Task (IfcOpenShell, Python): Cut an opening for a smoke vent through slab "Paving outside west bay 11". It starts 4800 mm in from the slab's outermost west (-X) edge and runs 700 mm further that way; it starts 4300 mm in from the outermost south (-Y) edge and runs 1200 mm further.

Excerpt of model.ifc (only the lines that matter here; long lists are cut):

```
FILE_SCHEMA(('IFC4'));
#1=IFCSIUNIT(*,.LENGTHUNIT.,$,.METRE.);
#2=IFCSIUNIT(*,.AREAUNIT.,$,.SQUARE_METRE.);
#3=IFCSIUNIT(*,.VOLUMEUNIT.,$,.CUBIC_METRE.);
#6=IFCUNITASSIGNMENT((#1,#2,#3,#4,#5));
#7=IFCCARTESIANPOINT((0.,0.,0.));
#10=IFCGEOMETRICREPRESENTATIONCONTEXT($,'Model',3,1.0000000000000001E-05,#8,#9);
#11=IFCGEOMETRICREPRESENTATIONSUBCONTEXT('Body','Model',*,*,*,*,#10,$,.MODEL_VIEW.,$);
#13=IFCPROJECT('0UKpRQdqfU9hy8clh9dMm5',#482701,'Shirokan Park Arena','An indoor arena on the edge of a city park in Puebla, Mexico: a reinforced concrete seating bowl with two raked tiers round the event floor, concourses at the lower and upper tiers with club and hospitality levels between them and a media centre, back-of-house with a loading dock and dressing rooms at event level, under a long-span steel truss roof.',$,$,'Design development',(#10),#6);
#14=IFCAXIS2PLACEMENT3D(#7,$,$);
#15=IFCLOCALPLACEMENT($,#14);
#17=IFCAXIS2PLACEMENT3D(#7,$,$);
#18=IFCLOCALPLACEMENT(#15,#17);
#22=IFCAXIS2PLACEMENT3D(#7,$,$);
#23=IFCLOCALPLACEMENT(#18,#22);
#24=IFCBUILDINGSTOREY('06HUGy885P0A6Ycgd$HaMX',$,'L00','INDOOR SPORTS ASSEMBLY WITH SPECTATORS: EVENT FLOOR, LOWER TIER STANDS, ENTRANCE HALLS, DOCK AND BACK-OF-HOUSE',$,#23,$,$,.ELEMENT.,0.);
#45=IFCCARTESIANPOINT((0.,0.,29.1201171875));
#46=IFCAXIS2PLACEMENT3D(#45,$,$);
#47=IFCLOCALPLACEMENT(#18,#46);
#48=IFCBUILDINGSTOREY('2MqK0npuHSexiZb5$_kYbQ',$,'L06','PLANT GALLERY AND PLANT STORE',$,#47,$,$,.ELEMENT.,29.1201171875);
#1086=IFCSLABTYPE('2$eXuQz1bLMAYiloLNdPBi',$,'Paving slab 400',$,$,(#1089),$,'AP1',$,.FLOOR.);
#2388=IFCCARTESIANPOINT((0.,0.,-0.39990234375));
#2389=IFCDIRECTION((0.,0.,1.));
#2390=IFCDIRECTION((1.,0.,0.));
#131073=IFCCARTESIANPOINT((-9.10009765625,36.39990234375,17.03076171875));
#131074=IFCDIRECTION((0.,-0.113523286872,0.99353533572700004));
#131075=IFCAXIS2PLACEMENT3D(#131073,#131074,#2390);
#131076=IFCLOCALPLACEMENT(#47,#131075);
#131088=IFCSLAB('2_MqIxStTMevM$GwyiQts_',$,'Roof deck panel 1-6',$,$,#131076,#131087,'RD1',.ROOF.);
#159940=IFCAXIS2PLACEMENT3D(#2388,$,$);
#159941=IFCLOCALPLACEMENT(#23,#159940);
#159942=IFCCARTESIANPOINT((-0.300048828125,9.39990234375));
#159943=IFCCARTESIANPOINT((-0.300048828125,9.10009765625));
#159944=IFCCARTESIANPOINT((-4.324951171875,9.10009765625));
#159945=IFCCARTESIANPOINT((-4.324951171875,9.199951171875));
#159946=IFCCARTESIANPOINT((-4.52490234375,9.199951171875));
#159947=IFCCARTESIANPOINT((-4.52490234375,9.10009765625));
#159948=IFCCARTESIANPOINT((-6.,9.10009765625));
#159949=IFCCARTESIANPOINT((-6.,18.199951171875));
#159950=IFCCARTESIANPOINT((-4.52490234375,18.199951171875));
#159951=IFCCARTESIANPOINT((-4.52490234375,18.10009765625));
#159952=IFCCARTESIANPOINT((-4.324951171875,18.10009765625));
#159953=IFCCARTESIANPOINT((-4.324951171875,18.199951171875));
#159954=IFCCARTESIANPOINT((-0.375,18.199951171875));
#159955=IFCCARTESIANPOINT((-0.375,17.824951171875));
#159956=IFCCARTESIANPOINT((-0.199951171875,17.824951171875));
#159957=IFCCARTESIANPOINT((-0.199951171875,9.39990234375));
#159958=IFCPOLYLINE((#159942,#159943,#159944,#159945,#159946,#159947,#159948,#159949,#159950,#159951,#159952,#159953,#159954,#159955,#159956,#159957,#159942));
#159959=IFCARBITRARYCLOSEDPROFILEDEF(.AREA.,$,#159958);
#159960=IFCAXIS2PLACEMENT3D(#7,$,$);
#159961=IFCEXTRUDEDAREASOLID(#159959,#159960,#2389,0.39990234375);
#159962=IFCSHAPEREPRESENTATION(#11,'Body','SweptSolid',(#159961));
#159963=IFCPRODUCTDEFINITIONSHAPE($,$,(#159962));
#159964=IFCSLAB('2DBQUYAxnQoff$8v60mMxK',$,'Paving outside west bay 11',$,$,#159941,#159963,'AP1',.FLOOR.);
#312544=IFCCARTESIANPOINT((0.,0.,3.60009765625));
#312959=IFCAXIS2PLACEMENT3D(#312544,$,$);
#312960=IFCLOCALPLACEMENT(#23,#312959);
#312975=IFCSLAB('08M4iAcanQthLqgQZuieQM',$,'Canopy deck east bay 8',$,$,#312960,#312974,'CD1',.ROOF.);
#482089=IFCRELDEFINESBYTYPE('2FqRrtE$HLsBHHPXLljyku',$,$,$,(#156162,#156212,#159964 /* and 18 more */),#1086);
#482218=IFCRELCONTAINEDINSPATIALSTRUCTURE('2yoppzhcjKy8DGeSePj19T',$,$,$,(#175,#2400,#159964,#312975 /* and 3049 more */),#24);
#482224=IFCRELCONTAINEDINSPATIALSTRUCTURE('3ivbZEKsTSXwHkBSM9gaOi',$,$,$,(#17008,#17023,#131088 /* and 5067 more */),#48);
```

```python
import numpy as np
import ifcopenshell
import ifcopenshell.api.feature
import ifcopenshell.api.geometry
import ifcopenshell.api.root
import ifcopenshell.geom
import ifcopenshell.util.placement
import ifcopenshell.util.representation
import ifcopenshell.util.shape
import ifcopenshell.util.unit

model = ifcopenshell.open("model.ifc")
unit_scale = ifcopenshell.util.unit.calculate_unit_scale(model)
settings = ifcopenshell.geom.settings()


def volume(element):
    """Net volume in cubic metres, openings subtracted."""
    shape = ifcopenshell.geom.create_shape(settings, element)
    return ifcopenshell.util.shape.get_volume(shape.geometry)


slab = model.by_id(159964)
before = volume(slab)

# Extent in the slab's own axes, in metres. The edges named are its -X and -Y sides.
slab_shape = ifcopenshell.geom.create_shape(settings, slab)
vertices = ifcopenshell.util.shape.get_vertices(slab_shape.geometry)
x_min, y_min, bottom = vertices.min(axis=0)
top = vertices[:, 2].max()

opening = ifcopenshell.api.root.create_entity(model, ifc_class="IfcOpeningElement", name="Smoke vent opening", predefined_type="OPENING")
context = ifcopenshell.util.representation.get_context(model, "Model", "Body", "MODEL_VIEW")
width, depth = 0.7, 1.2
outline = [(0.0, 0.0), (width, 0.0), (width, depth), (0.0, depth), (0.0, 0.0)]
# Overshoot both faces by 50 mm so the cut is clean.
shape = ifcopenshell.api.geometry.add_slab_representation(
    model, context=context, depth=top - bottom + 0.1, polyline=outline
)
ifcopenshell.api.geometry.assign_representation(model, product=opening, representation=shape)

matrix = ifcopenshell.util.placement.get_local_placement(slab.ObjectPlacement)
matrix[:, 3] = matrix @ np.append(np.array([x_min + 4.8, y_min + 4.3, bottom - 0.05]) / unit_scale, 1.0)
ifcopenshell.api.geometry.edit_object_placement(model, product=opening, matrix=matrix, is_si=False)
ifcopenshell.api.feature.add_feature(model, feature=opening, element=slab)

after = volume(slab)

print(f"slab volume {before:.3f} -> {after:.3f} m3")

model.write("model_rev.ifc")
```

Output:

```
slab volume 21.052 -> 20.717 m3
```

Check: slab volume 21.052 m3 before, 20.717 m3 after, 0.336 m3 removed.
